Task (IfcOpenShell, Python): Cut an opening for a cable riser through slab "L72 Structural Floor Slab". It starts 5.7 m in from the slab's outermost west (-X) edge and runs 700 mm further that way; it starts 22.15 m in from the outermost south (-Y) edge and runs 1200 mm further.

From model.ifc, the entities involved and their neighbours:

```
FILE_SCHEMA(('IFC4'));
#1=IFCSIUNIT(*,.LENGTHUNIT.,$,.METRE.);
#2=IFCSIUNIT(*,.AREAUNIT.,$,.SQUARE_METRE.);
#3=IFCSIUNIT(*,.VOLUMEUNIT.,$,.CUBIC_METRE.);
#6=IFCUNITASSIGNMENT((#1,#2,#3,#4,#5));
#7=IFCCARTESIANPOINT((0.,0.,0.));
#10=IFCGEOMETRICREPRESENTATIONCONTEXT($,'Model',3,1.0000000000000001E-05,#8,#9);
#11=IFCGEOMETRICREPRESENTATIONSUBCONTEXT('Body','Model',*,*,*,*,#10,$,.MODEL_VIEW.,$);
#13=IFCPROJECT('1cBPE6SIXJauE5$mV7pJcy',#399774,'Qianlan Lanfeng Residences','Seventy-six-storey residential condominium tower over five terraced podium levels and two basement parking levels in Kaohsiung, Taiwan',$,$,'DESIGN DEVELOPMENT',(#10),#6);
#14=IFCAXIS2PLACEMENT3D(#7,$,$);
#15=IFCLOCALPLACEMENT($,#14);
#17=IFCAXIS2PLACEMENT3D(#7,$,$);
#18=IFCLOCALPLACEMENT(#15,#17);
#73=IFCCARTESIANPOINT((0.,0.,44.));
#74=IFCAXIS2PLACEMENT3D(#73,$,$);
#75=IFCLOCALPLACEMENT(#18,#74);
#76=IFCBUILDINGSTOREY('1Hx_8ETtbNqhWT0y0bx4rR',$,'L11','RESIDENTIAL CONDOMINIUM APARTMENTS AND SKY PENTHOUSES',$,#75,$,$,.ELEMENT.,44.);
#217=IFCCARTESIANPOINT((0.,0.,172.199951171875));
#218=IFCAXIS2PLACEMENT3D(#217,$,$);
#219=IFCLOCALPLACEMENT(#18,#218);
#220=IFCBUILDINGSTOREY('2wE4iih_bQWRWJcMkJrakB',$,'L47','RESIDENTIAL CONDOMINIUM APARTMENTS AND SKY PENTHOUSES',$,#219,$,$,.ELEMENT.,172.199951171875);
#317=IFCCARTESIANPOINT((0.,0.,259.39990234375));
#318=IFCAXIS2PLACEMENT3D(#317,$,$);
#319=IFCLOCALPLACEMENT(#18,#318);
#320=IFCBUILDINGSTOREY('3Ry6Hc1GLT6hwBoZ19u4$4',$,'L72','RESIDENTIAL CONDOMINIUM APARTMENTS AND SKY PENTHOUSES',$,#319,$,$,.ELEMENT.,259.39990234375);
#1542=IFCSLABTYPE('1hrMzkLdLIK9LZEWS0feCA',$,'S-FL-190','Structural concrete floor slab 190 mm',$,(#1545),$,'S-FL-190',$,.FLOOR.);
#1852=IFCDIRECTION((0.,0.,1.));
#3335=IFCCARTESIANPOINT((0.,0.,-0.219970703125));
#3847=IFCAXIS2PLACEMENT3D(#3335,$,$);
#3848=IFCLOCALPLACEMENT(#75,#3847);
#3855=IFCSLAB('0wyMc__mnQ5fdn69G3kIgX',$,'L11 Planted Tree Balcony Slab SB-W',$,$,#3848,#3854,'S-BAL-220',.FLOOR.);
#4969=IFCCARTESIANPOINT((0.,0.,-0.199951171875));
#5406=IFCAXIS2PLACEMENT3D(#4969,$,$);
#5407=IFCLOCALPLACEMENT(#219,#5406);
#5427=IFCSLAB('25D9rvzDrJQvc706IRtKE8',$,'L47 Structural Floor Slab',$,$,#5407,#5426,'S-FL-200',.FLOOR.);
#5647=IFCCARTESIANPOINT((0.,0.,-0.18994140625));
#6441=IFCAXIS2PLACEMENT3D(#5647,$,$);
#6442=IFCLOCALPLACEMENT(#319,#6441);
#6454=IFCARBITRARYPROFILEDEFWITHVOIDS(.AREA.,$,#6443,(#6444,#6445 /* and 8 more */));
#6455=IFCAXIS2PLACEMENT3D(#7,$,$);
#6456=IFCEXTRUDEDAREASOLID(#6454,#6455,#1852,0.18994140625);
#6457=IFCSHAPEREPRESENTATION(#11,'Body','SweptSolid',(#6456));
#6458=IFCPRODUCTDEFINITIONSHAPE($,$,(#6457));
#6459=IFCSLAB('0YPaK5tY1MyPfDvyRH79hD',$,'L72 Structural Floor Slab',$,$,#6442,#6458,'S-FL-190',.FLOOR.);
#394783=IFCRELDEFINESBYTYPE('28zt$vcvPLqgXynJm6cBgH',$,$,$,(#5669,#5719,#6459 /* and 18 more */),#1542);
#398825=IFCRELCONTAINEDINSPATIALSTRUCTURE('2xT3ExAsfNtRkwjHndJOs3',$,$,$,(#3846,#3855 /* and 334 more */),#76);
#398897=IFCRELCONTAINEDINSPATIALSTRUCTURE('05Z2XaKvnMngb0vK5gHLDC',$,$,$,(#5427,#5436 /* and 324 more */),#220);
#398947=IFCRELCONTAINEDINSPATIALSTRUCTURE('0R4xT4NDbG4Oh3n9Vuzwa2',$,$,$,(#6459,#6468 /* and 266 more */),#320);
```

```python
import numpy as np
import ifcopenshell
import ifcopenshell.api.feature
import ifcopenshell.api.geometry
import ifcopenshell.api.root
import ifcopenshell.geom
import ifcopenshell.util.placement
import ifcopenshell.util.representation
import ifcopenshell.util.shape
import ifcopenshell.util.unit

model = ifcopenshell.open("model.ifc")
unit_scale = ifcopenshell.util.unit.calculate_unit_scale(model)
settings = ifcopenshell.geom.settings()


def volume(element):
    """Net volume in cubic metres, openings subtracted."""
    shape = ifcopenshell.geom.create_shape(settings, element)
    return ifcopenshell.util.shape.get_volume(shape.geometry)


slab = model.by_id(6459)
before = volume(slab)

# Extent in the slab's own axes, in metres. The edges named are its -X and -Y sides.
slab_shape = ifcopenshell.geom.create_shape(settings, slab)
vertices = ifcopenshell.util.shape.get_vertices(slab_shape.geometry)
x_min, y_min, bottom = vertices.min(axis=0)
top = vertices[:, 2].max()

opening = ifcopenshell.api.root.create_entity(model, ifc_class="IfcOpeningElement", name="Cable riser opening", predefined_type="OPENING")
context = ifcopenshell.util.representation.get_context(model, "Model", "Body", "MODEL_VIEW")
width, depth = 0.7, 1.2
outline = [(0.0, 0.0), (width, 0.0), (width, depth), (0.0, depth), (0.0, 0.0)]
# Overshoot both faces by 50 mm so the cut is clean.
shape = ifcopenshell.api.geometry.add_slab_representation(
    model, context=context, depth=top - bottom + 0.1, polyline=outline
)
ifcopenshell.api.geometry.assign_representation(model, product=opening, representation=shape)

matrix = ifcopenshell.util.placement.get_local_placement(slab.ObjectPlacement)
matrix[:, 3] = matrix @ np.append(np.array([x_min + 5.7, y_min + 22.15, bottom - 0.05]) / unit_scale, 1.0)
ifcopenshell.api.geometry.edit_object_placement(model, product=opening, matrix=matrix, is_si=False)
ifcopenshell.api.feature.add_feature(model, feature=opening, element=slab)

after = volume(slab)

print(f"slab volume {before:.3f} -> {after:.3f} m3")

model.write("model-out.ifc")
```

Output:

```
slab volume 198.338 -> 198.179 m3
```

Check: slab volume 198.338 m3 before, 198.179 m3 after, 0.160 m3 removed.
